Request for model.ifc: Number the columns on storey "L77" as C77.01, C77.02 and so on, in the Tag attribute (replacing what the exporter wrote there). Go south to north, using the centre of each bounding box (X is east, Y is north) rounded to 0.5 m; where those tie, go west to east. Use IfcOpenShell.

First a look at what the model holds.

```python
import ifcopenshell
import ifcopenshell.util.element
import ifcopenshell.util.placement

model = ifcopenshell.open("model.ifc")
print(model.schema)
storey = next(s for s in model.by_type("IfcBuildingStorey") if s.Name == "L77")
columns = [e for e in ifcopenshell.util.element.get_decomposition(storey) if e.is_a("IfcColumn")]
for e in sorted(columns, key=lambda e: e.id()):
    origin = ifcopenshell.util.placement.get_local_placement(e.ObjectPlacement)[:3, 3]
    print(e.id(), e.Tag, e.Name, origin.round(2) + 0.0, sep=" | ")
```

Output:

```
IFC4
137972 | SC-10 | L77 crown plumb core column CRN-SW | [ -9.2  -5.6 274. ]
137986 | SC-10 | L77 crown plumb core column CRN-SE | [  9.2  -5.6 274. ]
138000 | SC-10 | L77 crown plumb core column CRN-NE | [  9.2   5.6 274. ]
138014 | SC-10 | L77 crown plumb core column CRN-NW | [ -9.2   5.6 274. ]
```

```python
import ifcopenshell
import ifcopenshell.geom
import ifcopenshell.util.element
import ifcopenshell.util.shape

model = ifcopenshell.open("model.ifc")
settings = ifcopenshell.geom.settings()
settings.set("use-world-coords", True)


def centre(element):
    shape = ifcopenshell.geom.create_shape(settings, element)
    return ifcopenshell.util.shape.get_bbox_centroid(shape.geometry)


storey = next(s for s in model.by_type("IfcBuildingStorey") if s.Name == "L77")
columns = [e for e in ifcopenshell.util.element.get_decomposition(storey) if e.is_a("IfcColumn")]

# Insertion points can sit at a corner or the storey origin, so sort by the geometry (in metres).
centres = {e: centre(e) for e in columns}
columns.sort(key=lambda e: (round(centres[e][1] / 0.5), centres[e][0]))

for i, e in enumerate(columns, start=1):
    number = f"C77.{i:02d}"
    e.Tag = number
    print(e.id(), number)

model.write("model_v2.ifc")
```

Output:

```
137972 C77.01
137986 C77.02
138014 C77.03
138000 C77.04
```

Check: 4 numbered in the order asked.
